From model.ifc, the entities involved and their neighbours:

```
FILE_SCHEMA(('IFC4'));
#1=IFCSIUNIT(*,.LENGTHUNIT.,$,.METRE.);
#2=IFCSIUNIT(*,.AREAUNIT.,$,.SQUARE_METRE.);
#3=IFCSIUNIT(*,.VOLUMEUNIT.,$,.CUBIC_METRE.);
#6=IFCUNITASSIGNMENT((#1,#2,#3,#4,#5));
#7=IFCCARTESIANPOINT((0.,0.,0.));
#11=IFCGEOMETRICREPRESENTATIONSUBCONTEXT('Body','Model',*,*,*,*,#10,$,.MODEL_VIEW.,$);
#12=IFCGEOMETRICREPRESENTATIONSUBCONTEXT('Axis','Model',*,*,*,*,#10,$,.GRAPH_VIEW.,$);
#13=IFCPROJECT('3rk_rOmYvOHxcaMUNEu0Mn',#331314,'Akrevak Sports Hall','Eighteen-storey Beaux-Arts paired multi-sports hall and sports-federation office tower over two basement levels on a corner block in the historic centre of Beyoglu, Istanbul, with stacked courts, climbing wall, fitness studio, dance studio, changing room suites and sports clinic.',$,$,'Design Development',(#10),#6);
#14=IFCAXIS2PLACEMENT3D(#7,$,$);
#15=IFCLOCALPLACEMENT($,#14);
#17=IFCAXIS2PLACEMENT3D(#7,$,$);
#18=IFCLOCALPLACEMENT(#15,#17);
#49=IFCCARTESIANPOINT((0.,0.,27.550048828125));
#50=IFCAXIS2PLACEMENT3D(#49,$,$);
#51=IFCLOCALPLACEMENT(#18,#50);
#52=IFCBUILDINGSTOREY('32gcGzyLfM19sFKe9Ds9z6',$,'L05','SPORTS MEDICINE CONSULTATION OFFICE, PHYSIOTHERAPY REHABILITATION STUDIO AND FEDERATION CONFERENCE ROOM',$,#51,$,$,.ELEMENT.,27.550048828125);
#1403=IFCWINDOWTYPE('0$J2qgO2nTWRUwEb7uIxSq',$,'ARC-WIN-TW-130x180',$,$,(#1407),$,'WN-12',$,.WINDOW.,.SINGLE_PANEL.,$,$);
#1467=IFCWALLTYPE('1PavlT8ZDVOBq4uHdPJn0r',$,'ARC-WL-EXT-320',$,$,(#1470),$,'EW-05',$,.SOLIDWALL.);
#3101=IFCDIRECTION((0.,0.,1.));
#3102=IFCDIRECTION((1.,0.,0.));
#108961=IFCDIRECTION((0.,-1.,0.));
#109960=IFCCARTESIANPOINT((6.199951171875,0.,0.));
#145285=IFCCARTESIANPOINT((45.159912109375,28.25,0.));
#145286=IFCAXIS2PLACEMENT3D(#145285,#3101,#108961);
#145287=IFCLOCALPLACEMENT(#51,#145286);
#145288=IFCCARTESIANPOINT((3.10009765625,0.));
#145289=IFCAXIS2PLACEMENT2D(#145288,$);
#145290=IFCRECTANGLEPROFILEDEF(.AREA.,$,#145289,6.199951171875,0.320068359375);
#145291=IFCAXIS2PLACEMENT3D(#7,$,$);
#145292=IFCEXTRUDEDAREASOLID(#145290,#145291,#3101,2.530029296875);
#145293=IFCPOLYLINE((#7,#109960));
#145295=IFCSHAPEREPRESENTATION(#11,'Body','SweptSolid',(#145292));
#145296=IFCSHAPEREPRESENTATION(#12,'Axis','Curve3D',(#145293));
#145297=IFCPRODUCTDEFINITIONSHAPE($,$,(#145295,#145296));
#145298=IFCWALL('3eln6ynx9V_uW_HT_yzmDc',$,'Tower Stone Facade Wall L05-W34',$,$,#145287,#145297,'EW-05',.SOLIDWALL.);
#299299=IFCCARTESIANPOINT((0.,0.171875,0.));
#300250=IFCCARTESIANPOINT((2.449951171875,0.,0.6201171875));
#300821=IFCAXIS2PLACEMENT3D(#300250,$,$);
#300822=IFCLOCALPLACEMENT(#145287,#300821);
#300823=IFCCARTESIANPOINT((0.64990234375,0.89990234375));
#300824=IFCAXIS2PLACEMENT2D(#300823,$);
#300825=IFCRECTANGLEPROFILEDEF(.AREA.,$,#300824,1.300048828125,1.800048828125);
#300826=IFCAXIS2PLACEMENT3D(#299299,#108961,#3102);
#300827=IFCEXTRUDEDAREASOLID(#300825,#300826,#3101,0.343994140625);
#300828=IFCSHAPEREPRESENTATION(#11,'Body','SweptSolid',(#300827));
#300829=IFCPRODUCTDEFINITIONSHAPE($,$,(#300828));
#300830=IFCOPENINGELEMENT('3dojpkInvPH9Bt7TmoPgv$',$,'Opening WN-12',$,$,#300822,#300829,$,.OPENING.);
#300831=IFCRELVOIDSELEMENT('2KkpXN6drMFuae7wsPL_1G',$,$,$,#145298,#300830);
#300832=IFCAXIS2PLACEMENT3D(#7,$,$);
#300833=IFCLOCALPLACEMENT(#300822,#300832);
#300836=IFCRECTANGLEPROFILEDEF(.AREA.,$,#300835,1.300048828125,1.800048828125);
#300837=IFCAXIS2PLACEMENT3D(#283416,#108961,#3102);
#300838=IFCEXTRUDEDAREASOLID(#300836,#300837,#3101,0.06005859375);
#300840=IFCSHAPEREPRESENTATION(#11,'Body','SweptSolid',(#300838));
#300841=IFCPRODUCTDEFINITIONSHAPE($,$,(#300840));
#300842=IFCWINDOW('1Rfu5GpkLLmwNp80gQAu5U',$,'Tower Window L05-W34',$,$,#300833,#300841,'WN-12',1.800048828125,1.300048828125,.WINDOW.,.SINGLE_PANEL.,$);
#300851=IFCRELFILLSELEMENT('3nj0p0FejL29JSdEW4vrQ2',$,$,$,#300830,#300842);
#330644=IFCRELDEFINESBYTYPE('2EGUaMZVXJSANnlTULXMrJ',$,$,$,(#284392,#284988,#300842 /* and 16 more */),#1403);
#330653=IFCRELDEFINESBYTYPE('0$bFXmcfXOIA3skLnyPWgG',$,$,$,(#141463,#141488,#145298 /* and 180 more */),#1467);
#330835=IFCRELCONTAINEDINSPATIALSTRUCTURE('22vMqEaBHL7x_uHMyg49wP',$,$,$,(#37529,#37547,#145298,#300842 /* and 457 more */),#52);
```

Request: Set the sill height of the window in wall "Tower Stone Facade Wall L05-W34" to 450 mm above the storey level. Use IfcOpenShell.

```python
import numpy as np
import ifcopenshell
import ifcopenshell.api.geometry
import ifcopenshell.geom
import ifcopenshell.util.element
import ifcopenshell.util.placement
import ifcopenshell.util.shape
import ifcopenshell.util.unit

model = ifcopenshell.open("model.ifc")
unit_scale = ifcopenshell.util.unit.calculate_unit_scale(model)

window = model.by_id(300842)
opening = window.FillsVoids[0].RelatingOpeningElement
storey = ifcopenshell.util.element.get_container(window, ifc_class="IfcBuildingStorey")
level = ifcopenshell.util.placement.get_local_placement(storey.ObjectPlacement)[2, 3]

# The opening's origin need not be at the sill, so measure its lowest point.
shape = ifcopenshell.geom.create_shape(ifcopenshell.geom.settings(), opening)
bottom = ifcopenshell.util.shape.get_shape_bottom_elevation(shape, shape.geometry) / unit_scale
dz = level + 0.45 / unit_scale - bottom

shift = np.array([0.0, 0.0, dz])
# The window is placed relative to its opening, so it follows when the opening moves.
matrix = ifcopenshell.util.placement.get_local_placement(opening.ObjectPlacement)
matrix[:3, 3] += shift
ifcopenshell.api.geometry.edit_object_placement(
    model, product=opening, matrix=matrix, is_si=False, should_transform_children=True
)

print(f"moved by {dz * unit_scale:+.3f} m")

model.write("model_rev.ifc")
```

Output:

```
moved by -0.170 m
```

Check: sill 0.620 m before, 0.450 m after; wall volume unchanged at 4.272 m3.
